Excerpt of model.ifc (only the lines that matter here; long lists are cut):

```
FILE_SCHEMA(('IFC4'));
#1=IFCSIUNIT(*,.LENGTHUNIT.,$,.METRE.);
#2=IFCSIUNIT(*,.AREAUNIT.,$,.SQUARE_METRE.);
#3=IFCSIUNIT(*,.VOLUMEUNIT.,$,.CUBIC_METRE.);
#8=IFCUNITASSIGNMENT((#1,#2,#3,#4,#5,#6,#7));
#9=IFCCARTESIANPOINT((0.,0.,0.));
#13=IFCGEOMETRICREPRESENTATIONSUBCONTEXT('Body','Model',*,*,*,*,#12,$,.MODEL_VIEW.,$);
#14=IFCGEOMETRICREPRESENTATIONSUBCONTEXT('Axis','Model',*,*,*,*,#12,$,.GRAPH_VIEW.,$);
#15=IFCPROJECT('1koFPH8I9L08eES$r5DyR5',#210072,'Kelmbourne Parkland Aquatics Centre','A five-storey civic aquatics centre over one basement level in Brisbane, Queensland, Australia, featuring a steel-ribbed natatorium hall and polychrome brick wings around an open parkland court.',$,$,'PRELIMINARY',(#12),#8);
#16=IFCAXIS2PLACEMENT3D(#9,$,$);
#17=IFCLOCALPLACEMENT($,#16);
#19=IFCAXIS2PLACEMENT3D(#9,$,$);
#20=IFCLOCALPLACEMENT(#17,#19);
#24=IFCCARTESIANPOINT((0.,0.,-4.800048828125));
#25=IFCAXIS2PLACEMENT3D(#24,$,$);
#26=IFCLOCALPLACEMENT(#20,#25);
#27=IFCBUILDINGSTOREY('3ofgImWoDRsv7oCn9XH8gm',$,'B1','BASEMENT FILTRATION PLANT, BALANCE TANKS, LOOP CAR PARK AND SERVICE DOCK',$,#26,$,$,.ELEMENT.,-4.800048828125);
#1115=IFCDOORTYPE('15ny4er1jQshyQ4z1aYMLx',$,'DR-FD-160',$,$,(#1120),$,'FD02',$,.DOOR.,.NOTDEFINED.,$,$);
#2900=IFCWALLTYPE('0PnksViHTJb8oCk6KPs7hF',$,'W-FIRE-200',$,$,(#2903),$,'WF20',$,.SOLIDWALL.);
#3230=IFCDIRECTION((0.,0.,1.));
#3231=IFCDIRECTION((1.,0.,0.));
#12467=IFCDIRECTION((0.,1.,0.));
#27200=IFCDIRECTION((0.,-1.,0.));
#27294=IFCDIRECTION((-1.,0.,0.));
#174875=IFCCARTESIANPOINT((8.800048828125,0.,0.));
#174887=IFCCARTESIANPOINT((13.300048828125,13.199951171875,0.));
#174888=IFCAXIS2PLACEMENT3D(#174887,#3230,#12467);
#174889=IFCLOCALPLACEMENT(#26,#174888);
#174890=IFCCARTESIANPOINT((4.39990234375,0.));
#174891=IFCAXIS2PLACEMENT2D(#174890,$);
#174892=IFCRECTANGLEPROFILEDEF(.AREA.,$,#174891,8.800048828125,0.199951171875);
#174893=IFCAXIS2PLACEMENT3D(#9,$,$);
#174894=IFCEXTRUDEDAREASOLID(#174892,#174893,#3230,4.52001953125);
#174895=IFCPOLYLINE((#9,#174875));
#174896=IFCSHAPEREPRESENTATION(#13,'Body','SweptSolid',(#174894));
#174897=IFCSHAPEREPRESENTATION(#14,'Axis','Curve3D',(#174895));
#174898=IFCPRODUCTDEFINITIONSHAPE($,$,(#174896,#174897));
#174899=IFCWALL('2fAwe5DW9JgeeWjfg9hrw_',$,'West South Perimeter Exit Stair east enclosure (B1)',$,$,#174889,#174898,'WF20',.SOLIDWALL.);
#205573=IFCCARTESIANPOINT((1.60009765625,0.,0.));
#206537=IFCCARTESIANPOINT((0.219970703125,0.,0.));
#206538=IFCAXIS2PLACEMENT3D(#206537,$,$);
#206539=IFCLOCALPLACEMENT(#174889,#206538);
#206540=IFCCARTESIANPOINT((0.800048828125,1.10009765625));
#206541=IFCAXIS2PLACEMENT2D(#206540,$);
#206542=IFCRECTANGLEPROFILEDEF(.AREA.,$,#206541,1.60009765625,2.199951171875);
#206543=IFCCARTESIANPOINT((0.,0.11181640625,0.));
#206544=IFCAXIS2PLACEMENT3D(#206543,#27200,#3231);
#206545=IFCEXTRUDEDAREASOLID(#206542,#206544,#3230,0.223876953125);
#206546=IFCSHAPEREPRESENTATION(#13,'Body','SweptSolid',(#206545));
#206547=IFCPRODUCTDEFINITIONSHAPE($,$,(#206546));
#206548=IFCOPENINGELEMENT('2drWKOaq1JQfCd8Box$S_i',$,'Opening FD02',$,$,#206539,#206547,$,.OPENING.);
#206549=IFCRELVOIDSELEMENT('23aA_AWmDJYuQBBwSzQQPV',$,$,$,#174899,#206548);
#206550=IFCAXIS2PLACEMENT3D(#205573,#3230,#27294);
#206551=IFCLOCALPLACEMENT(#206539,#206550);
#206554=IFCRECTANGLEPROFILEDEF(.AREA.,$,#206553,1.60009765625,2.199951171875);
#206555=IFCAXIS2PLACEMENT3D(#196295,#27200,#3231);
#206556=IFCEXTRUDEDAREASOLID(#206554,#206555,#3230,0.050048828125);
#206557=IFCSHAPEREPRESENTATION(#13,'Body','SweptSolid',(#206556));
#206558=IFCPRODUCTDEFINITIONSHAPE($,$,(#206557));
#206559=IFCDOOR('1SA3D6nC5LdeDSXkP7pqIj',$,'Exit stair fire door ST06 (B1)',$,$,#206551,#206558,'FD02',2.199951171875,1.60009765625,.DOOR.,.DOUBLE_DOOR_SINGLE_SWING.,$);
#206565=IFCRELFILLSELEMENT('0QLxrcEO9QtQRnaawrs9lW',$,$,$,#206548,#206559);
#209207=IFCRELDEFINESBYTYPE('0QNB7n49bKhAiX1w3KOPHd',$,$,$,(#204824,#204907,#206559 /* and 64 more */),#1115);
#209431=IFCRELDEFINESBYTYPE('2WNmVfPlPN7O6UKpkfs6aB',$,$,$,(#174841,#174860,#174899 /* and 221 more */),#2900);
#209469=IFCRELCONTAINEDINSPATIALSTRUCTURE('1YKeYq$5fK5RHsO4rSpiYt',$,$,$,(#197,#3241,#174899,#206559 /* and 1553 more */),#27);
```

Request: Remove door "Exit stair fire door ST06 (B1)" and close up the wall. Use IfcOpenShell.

```python
import ifcopenshell
import ifcopenshell.api.feature
import ifcopenshell.api.root
import ifcopenshell.geom
import ifcopenshell.util.shape

model = ifcopenshell.open("model.ifc")
settings = ifcopenshell.geom.settings()


def volume(element):
    """Net volume in cubic metres, openings subtracted."""
    shape = ifcopenshell.geom.create_shape(settings, element)
    return ifcopenshell.util.shape.get_volume(shape.geometry)


door = model.by_id(206559)
opening = door.FillsVoids[0].RelatingOpeningElement
wall = opening.VoidsElements[0].RelatingBuildingElement
before = volume(wall)

ifcopenshell.api.root.remove_product(model, product=door)
ifcopenshell.api.feature.remove_feature(model, feature=opening)

after = volume(wall)

print(f"wall volume {before:.3f} -> {after:.3f} m3")

model.write("model_updated.ifc")
```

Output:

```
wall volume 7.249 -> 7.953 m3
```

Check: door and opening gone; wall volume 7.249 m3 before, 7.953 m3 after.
